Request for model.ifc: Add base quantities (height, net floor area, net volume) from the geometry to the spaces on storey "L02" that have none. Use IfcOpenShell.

First a look at what the model holds.

```python
import ifcopenshell
import ifcopenshell.util.element
import ifcopenshell.util.unit

model = ifcopenshell.open("model.ifc")
print(model.schema)
for unit_type in ("LENGTHUNIT", "AREAUNIT", "VOLUMEUNIT"):
    print(unit_type, ifcopenshell.util.unit.calculate_unit_scale(model, unit_type))
storey = next(s for s in model.by_type("IfcBuildingStorey") if s.Name == "L02")
spaces = [e for e in ifcopenshell.util.element.get_decomposition(storey) if e.is_a("IfcSpace")]
for e in sorted(spaces, key=lambda e: e.id()):
    print(e.id(), e.is_a(), e.Name, list(ifcopenshell.util.element.get_psets(e, qtos_only=True)), sep=" | ")
```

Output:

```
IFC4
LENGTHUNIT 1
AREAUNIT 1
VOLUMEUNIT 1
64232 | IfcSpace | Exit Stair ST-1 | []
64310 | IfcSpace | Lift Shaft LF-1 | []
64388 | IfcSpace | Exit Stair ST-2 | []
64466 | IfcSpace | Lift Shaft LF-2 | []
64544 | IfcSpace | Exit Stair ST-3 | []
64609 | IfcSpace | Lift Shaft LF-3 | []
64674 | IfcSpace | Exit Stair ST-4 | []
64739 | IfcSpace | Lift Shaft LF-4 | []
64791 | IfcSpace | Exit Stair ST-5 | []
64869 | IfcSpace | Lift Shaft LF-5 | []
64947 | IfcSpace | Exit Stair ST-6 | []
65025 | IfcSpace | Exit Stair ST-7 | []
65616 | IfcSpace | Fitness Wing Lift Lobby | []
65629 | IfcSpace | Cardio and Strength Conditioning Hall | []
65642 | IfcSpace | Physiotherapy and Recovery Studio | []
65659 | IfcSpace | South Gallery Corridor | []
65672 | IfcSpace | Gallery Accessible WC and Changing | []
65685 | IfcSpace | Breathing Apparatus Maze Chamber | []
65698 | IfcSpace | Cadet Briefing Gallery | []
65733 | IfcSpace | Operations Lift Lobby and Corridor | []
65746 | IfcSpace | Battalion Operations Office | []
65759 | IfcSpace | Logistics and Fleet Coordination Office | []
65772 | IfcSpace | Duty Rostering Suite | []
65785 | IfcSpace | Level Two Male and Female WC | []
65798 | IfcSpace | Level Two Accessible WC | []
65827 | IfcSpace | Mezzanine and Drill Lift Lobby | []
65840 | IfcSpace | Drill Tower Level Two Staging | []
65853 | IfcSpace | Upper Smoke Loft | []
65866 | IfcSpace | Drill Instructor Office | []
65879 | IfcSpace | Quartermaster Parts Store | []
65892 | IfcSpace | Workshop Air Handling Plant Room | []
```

```python
import ifcopenshell
import ifcopenshell.api.pset
import ifcopenshell.geom
import ifcopenshell.util.element
import ifcopenshell.util.shape
import ifcopenshell.util.unit

model = ifcopenshell.open("model.ifc")
unit_scale = ifcopenshell.util.unit.calculate_unit_scale(model)
area_scale = ifcopenshell.util.unit.calculate_unit_scale(model, "AREAUNIT")
volume_scale = ifcopenshell.util.unit.calculate_unit_scale(model, "VOLUMEUNIT")
settings = ifcopenshell.geom.settings()

storey = next(s for s in model.by_type("IfcBuildingStorey") if s.Name == "L02")
spaces = [e for e in ifcopenshell.util.element.get_decomposition(storey) if e.is_a("IfcSpace")]

for e in sorted(spaces, key=lambda e: e.id()):
    if ifcopenshell.util.element.get_psets(e, qtos_only=True, should_inherit=False):
        continue
    # Geometry comes back in metres, in the element's own axes.
    shape = ifcopenshell.geom.create_shape(settings, e)
    values = {
        "Height": ifcopenshell.util.shape.get_z(shape.geometry) / unit_scale,
        "NetFloorArea": ifcopenshell.util.shape.get_footprint_area(shape.geometry) / area_scale,
        "NetVolume": ifcopenshell.util.shape.get_volume(shape.geometry) / volume_scale,
    }
    qto = ifcopenshell.api.pset.add_qto(model, product=e, name="Qto_SpaceBaseQuantities")
    ifcopenshell.api.pset.edit_qto(model, qto=qto, properties=values)
    print(e.id(), {k: round(v, 3) for k, v in values.items()})

model.write("model_rev.ifc")
```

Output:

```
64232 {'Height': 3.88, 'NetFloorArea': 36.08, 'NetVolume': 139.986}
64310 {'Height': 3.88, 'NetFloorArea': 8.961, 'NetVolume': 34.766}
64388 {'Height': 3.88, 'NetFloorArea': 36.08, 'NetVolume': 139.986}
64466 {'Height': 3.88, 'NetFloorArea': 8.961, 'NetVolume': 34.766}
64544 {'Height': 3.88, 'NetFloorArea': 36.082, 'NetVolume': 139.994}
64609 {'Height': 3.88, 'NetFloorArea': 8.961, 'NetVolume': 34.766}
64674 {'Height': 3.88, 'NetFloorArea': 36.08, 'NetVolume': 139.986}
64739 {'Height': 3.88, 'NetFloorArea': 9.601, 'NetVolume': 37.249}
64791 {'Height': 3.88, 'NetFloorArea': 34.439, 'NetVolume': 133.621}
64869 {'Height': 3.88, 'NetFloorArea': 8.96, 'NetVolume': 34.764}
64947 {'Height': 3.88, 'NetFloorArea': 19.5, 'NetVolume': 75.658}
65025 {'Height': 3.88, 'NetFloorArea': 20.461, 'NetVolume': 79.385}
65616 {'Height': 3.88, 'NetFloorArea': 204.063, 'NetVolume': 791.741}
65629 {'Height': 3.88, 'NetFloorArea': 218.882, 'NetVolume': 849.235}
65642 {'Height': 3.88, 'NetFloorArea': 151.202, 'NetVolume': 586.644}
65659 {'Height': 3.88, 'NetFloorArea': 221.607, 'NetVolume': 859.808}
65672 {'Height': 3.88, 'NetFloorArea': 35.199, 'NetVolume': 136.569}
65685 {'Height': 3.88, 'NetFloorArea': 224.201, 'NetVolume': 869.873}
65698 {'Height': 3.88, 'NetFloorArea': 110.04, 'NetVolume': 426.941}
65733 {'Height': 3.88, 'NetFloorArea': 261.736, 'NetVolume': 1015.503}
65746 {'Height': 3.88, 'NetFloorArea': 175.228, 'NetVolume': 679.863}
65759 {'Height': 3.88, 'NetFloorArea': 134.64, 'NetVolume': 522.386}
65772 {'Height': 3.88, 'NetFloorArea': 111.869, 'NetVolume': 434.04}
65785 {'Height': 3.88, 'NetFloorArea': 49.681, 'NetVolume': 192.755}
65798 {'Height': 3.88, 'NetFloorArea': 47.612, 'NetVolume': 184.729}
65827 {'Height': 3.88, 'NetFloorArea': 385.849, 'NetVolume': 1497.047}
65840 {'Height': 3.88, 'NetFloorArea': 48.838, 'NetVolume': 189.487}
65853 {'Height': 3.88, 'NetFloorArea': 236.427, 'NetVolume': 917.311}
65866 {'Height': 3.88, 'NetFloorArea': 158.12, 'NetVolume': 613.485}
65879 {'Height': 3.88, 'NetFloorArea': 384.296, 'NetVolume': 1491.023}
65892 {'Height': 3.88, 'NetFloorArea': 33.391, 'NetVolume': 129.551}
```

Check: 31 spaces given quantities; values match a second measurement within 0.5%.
